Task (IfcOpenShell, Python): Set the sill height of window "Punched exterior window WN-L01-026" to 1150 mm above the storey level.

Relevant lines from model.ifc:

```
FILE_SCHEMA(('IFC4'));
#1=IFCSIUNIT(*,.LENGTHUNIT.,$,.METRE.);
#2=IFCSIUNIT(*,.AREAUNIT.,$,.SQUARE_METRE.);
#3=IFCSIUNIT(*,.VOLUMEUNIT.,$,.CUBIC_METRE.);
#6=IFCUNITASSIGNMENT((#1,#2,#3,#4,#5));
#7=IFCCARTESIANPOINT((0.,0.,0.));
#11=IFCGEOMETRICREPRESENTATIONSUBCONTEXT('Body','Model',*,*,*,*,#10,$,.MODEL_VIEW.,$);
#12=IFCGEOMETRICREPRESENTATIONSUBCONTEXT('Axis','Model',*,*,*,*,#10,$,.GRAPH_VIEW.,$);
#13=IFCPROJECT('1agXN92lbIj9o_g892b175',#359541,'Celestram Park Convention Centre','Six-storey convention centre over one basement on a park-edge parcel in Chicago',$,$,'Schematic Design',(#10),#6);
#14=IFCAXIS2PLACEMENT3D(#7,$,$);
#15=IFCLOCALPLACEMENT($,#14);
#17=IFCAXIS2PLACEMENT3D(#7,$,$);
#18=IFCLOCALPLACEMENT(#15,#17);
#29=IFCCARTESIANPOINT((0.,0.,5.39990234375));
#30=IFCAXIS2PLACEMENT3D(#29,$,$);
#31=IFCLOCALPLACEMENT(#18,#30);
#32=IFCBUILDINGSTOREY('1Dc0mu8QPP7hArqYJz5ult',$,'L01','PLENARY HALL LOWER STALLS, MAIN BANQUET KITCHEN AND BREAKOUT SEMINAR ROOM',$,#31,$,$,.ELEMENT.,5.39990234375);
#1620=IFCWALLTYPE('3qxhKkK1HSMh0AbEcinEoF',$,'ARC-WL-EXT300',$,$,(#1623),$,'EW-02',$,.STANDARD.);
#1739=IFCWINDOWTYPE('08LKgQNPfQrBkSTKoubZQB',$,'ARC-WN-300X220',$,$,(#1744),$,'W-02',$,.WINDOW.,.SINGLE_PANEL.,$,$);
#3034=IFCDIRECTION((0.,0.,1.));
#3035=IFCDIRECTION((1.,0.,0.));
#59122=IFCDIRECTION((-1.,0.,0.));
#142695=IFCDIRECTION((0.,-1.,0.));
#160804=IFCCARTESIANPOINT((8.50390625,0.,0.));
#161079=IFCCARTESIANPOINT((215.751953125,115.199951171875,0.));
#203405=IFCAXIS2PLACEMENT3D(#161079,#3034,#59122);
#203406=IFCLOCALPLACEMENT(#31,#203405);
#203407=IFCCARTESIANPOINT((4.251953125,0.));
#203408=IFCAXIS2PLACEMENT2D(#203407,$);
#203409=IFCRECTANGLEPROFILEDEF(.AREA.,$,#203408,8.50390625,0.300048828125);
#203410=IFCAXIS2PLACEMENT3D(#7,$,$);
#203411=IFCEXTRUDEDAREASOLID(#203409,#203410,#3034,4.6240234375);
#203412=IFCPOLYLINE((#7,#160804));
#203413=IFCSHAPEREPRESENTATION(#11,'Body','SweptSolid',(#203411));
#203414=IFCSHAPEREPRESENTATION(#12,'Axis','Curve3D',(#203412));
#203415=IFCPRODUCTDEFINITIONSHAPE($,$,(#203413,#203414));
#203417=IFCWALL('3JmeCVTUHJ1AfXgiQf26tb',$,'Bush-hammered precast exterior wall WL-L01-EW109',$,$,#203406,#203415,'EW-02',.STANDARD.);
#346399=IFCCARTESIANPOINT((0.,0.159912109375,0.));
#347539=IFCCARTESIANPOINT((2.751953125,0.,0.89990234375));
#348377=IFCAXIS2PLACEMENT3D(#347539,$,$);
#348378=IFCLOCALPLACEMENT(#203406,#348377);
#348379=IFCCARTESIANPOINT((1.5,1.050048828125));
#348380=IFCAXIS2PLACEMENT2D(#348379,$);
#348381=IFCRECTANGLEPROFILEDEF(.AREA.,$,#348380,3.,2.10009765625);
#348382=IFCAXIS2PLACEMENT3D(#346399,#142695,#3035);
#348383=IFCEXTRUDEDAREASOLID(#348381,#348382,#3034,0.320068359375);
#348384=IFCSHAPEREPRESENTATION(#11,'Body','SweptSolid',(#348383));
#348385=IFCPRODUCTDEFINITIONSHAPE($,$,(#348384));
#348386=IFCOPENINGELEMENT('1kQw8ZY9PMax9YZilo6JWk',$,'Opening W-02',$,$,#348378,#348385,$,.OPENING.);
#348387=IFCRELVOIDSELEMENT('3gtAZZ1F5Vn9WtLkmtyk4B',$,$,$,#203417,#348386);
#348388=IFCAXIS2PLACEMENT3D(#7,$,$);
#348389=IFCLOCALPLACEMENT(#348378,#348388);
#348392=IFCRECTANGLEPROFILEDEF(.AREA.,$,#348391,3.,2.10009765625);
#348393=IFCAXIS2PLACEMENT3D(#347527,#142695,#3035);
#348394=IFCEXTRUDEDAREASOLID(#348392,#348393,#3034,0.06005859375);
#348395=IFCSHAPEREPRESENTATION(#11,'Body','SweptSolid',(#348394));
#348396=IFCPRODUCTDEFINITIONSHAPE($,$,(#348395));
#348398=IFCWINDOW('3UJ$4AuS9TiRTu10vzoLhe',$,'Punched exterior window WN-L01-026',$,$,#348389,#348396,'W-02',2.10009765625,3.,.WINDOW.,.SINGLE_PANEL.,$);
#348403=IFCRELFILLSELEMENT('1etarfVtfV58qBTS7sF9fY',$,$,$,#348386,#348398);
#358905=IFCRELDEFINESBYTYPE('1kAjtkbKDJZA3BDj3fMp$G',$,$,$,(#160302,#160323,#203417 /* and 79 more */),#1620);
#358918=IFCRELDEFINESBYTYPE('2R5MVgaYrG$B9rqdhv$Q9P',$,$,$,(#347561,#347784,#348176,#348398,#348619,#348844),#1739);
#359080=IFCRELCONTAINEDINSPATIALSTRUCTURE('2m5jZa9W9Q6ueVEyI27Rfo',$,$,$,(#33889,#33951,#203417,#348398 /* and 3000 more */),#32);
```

```python
import numpy as np
import ifcopenshell
import ifcopenshell.api.geometry
import ifcopenshell.geom
import ifcopenshell.util.element
import ifcopenshell.util.placement
import ifcopenshell.util.shape
import ifcopenshell.util.unit

model = ifcopenshell.open("model.ifc")
unit_scale = ifcopenshell.util.unit.calculate_unit_scale(model)

window = model.by_guid("3UJ$4AuS9TiRTu10vzoLhe")
opening = window.FillsVoids[0].RelatingOpeningElement
storey = ifcopenshell.util.element.get_container(window, ifc_class="IfcBuildingStorey")
level = ifcopenshell.util.placement.get_local_placement(storey.ObjectPlacement)[2, 3]

# The opening's origin need not be at the sill, so measure its lowest point.
shape = ifcopenshell.geom.create_shape(ifcopenshell.geom.settings(), opening)
bottom = ifcopenshell.util.shape.get_shape_bottom_elevation(shape, shape.geometry) / unit_scale
dz = level + 1.15 / unit_scale - bottom

shift = np.array([0.0, 0.0, dz])
# The window is placed relative to its opening, so it follows when the opening moves.
matrix = ifcopenshell.util.placement.get_local_placement(opening.ObjectPlacement)
matrix[:3, 3] += shift
ifcopenshell.api.geometry.edit_object_placement(
    model, product=opening, matrix=matrix, is_si=False, should_transform_children=True
)

print(f"moved by {dz * unit_scale:+.3f} m")

model.write("model-out.ifc")
```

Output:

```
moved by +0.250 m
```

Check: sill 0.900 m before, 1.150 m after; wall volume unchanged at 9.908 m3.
